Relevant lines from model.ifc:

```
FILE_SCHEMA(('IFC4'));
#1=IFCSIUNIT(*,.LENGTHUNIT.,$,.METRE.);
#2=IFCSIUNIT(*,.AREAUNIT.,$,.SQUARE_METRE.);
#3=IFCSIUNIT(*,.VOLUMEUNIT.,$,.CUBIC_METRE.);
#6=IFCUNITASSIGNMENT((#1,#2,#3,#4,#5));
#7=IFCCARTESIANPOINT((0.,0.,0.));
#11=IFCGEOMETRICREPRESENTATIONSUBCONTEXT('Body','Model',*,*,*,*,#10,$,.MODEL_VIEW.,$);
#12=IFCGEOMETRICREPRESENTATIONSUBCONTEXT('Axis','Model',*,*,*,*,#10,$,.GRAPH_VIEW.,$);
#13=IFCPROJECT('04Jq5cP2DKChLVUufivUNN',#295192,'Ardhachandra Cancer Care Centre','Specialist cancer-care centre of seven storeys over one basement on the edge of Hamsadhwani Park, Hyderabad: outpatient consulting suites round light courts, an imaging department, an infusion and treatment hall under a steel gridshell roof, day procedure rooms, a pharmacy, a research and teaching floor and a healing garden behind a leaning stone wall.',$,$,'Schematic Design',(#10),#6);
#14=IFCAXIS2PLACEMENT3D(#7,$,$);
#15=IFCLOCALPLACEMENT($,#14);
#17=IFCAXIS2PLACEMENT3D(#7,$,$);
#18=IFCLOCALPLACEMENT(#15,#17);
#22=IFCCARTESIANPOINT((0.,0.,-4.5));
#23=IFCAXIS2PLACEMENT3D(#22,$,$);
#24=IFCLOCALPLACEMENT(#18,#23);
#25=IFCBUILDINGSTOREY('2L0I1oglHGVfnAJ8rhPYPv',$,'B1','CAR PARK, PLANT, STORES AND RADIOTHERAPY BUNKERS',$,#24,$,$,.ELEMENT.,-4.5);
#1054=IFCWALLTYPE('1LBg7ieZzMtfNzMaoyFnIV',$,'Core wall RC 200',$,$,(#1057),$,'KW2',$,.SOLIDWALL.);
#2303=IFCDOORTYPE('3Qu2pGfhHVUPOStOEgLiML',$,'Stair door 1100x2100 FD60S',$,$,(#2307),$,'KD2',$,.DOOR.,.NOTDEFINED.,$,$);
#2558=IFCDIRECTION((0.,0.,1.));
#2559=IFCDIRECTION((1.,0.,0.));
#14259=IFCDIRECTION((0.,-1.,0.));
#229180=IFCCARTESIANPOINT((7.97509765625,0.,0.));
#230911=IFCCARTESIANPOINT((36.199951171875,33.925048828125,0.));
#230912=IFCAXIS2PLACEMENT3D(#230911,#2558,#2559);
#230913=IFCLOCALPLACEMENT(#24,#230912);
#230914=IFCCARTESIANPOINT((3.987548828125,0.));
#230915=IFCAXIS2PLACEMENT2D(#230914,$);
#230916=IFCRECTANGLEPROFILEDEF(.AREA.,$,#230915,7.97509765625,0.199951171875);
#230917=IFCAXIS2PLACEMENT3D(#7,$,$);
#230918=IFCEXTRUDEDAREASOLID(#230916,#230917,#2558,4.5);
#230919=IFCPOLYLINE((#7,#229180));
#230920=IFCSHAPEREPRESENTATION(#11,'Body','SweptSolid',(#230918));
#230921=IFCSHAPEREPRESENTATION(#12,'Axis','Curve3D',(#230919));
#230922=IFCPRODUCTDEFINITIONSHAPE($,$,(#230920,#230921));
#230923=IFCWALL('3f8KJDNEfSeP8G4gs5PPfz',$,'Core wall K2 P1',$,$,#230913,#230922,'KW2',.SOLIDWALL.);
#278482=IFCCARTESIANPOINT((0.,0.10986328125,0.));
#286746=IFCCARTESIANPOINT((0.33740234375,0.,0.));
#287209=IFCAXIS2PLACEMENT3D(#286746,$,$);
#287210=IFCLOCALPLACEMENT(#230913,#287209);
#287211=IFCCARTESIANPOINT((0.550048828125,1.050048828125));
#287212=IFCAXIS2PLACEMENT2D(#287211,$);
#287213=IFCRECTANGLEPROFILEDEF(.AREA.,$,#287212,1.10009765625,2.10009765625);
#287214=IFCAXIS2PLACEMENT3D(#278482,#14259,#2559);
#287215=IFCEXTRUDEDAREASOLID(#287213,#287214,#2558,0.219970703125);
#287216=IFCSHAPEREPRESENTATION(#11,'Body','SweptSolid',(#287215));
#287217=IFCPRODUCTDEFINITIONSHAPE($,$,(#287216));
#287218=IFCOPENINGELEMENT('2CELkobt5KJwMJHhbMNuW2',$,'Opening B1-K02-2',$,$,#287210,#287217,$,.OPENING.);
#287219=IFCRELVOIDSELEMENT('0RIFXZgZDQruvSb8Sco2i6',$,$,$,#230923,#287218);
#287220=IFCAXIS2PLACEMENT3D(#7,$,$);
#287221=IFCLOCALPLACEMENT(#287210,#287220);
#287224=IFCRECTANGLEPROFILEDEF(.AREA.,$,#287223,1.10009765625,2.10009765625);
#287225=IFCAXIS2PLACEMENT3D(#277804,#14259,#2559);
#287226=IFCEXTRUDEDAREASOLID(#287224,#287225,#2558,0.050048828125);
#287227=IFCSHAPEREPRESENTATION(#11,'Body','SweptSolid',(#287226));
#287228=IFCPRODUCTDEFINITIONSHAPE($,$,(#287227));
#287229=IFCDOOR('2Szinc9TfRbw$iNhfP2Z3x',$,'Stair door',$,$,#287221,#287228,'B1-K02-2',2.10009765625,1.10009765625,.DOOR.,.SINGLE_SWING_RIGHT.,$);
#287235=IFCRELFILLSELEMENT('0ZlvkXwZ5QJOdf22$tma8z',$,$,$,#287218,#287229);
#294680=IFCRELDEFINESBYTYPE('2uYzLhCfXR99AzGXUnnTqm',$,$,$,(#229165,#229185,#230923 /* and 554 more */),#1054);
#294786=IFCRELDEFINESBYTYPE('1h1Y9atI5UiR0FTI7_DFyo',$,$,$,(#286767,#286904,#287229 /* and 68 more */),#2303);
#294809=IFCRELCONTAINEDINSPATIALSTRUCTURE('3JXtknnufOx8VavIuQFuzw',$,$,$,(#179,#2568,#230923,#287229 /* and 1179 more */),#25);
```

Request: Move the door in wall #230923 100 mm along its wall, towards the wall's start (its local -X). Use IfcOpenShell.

```python
import ifcopenshell
import ifcopenshell.api.geometry
import ifcopenshell.util.placement
import ifcopenshell.util.unit

model = ifcopenshell.open("model.ifc")
unit_scale = ifcopenshell.util.unit.calculate_unit_scale(model)

door = model.by_id(287229)
opening = door.FillsVoids[0].RelatingOpeningElement
wall = opening.VoidsElements[0].RelatingBuildingElement

wall_matrix = ifcopenshell.util.placement.get_local_placement(wall.ObjectPlacement)
shift = wall_matrix[:3, 0] * -0.1 / unit_scale
before = ifcopenshell.util.placement.get_local_placement(door.ObjectPlacement)[:3, 3].copy()

# The door is placed relative to its opening, so it follows when the opening moves.
matrix = ifcopenshell.util.placement.get_local_placement(opening.ObjectPlacement)
matrix[:3, 3] += shift
ifcopenshell.api.geometry.edit_object_placement(
    model, product=opening, matrix=matrix, is_si=False, should_transform_children=True
)

after = ifcopenshell.util.placement.get_local_placement(door.ObjectPlacement)[:3, 3]
print("door moved by", (after - before).round(3) + 0.0)

model.write("model-out.ifc")
```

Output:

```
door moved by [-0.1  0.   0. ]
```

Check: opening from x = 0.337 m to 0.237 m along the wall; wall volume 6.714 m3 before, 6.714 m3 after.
